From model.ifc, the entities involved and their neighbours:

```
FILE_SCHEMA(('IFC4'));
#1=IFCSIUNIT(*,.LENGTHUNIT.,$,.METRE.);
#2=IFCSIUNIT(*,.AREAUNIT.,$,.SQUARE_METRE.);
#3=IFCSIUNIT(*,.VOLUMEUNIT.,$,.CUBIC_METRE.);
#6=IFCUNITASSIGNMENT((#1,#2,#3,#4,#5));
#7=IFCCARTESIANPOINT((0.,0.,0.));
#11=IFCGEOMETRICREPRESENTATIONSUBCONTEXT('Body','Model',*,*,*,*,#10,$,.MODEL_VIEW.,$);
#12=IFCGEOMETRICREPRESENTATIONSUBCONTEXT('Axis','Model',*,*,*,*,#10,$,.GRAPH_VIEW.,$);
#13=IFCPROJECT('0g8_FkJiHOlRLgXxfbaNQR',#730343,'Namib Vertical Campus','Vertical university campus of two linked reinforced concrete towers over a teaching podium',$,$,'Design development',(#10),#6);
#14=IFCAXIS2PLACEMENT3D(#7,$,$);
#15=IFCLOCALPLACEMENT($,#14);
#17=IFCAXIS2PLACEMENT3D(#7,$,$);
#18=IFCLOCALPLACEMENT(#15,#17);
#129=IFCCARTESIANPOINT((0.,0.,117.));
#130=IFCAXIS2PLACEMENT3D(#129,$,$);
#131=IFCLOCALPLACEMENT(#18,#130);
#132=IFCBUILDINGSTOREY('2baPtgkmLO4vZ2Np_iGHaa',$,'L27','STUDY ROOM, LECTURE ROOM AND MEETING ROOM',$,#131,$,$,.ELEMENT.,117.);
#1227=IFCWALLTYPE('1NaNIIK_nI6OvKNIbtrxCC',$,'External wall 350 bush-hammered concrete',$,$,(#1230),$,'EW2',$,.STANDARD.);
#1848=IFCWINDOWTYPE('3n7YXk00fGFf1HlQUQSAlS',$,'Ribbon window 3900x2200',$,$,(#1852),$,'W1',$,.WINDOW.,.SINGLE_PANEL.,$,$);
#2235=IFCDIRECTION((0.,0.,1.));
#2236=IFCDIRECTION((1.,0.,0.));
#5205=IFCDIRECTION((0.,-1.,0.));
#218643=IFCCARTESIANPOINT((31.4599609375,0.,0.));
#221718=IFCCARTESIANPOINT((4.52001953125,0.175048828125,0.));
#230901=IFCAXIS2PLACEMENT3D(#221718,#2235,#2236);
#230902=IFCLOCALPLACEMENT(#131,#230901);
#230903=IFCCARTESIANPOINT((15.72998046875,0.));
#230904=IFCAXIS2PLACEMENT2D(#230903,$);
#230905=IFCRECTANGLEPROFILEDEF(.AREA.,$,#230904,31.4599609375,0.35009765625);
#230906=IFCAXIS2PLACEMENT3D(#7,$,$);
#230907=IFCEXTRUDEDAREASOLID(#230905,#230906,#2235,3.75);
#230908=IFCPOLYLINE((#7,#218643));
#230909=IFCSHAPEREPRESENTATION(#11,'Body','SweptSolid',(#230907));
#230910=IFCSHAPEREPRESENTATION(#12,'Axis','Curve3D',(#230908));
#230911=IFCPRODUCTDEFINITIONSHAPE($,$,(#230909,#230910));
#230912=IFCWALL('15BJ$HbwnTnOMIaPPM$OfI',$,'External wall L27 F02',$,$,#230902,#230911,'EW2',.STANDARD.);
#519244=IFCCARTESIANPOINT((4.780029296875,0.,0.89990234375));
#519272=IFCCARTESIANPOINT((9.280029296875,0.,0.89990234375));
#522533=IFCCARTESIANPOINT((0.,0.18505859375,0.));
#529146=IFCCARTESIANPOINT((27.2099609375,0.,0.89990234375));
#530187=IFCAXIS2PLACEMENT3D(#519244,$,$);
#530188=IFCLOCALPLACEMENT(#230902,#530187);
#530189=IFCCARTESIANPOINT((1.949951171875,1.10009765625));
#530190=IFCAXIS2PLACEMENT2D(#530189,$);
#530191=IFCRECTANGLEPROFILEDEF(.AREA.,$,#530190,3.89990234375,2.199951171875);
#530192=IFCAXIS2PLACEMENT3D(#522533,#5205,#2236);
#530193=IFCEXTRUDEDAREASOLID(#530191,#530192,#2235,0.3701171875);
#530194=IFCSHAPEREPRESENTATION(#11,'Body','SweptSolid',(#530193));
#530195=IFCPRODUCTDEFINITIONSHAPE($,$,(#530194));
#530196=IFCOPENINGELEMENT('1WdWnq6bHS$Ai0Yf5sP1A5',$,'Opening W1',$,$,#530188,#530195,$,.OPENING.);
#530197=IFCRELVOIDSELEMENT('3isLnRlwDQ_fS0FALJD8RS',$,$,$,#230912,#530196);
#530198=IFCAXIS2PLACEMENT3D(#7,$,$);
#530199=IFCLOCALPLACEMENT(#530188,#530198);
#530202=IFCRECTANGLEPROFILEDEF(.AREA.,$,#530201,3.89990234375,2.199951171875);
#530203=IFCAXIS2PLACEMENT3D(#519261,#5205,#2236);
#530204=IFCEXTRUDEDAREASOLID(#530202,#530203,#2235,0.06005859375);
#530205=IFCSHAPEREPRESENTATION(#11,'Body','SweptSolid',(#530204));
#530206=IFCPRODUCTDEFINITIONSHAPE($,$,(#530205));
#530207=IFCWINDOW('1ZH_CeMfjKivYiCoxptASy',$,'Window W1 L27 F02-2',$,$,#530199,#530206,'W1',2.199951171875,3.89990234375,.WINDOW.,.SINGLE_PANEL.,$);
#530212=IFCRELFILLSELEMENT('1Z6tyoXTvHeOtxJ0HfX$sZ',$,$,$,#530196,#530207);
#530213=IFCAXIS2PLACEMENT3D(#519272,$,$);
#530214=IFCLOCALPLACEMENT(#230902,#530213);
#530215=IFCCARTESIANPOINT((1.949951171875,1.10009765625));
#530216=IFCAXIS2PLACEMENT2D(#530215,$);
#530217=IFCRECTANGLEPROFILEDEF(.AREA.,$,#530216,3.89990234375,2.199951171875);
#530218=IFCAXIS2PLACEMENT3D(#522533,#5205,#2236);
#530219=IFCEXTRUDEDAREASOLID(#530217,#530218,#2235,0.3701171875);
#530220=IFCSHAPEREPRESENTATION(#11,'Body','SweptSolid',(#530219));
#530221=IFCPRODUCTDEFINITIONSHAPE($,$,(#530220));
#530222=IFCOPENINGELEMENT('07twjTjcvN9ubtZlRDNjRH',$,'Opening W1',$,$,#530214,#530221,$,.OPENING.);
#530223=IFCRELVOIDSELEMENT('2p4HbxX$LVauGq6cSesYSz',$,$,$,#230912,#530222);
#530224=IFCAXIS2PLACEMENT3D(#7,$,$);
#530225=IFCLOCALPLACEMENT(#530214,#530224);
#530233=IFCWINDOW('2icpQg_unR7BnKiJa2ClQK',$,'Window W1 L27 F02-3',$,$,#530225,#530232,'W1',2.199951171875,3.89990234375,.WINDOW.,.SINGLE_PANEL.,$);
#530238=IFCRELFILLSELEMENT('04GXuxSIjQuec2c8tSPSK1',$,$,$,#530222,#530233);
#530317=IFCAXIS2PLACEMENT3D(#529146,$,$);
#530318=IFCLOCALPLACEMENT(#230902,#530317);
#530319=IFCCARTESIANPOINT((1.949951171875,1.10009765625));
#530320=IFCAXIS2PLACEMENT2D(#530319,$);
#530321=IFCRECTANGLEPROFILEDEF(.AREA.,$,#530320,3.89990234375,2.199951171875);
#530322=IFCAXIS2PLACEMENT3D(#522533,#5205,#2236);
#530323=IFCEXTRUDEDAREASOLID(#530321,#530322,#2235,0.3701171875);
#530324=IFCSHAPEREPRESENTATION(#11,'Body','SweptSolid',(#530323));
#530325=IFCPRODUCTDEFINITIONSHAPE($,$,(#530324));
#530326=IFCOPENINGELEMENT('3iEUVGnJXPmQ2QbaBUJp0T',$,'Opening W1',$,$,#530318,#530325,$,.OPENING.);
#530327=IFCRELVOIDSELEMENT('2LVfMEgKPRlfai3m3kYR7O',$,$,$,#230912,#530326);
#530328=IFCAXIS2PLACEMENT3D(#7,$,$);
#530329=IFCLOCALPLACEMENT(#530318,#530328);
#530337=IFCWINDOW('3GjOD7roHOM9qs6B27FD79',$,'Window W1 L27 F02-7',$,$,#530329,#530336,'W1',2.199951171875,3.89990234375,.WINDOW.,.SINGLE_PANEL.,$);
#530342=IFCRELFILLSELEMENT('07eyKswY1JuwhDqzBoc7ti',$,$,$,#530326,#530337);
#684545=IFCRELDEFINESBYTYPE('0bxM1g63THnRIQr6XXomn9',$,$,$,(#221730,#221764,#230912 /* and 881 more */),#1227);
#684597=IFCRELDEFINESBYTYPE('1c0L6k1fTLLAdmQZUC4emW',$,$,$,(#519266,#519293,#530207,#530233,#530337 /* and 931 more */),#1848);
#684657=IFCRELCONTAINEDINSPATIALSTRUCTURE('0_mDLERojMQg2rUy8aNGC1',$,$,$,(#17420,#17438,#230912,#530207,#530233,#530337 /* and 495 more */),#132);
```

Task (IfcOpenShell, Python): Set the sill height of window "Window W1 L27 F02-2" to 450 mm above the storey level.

```python
import numpy as np
import ifcopenshell
import ifcopenshell.api.geometry
import ifcopenshell.geom
import ifcopenshell.util.element
import ifcopenshell.util.placement
import ifcopenshell.util.shape
import ifcopenshell.util.unit

model = ifcopenshell.open("model.ifc")
unit_scale = ifcopenshell.util.unit.calculate_unit_scale(model)

window = model.by_id(530207)
opening = window.FillsVoids[0].RelatingOpeningElement
storey = ifcopenshell.util.element.get_container(window, ifc_class="IfcBuildingStorey")
level = ifcopenshell.util.placement.get_local_placement(storey.ObjectPlacement)[2, 3]

# The opening's origin need not be at the sill, so measure its lowest point.
shape = ifcopenshell.geom.create_shape(ifcopenshell.geom.settings(), opening)
bottom = ifcopenshell.util.shape.get_shape_bottom_elevation(shape, shape.geometry) / unit_scale
dz = level + 0.45 - bottom

shift = np.array([0.0, 0.0, dz])
# The window is placed relative to its opening, so it follows when the opening moves.
matrix = ifcopenshell.util.placement.get_local_placement(opening.ObjectPlacement)
matrix[:3, 3] += shift
ifcopenshell.api.geometry.edit_object_placement(
    model, product=opening, matrix=matrix, is_si=False, should_transform_children=True
)

print(f"moved by {dz * unit_scale:+.3f} m")

model.write("model_v2.ifc")
```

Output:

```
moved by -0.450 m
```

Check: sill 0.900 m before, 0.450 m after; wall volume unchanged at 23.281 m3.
